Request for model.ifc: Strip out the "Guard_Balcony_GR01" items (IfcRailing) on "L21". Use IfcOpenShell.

First a look at what the model holds.

```python
import ifcopenshell
import ifcopenshell.util.element

model = ifcopenshell.open("model.ifc")
print(model.schema)
storey = next(s for s in model.by_type("IfcBuildingStorey") if s.Name == "L21")
railings = [e for e in ifcopenshell.util.element.get_decomposition(storey) if e.is_a("IfcRailing")]
seen = {}
for e in railings:
    element_type = ifcopenshell.util.element.get_type(e)
    name = element_type.Name if element_type not in (None, e) else None
    seen[name] = seen.get(name, 0) + 1
for name, count in sorted(seen.items(), key=str):
    print(count, "x", name)
```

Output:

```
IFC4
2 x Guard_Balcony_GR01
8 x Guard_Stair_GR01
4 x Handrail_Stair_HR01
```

```python
import ifcopenshell
import ifcopenshell.api.root
import ifcopenshell.util.element

model = ifcopenshell.open("model.ifc")

storey = next(s for s in model.by_type("IfcBuildingStorey") if s.Name == "L21")
railings = [e for e in ifcopenshell.util.element.get_decomposition(storey) if e.is_a("IfcRailing")]
targets = [e for e in railings if (t := ifcopenshell.util.element.get_type(e)) not in (None, e) and t.Name == "Guard_Balcony_GR01"]

for e in targets:
    ifcopenshell.api.root.remove_product(model, product=e)
print(len(targets), "removed")

model.write("model_edited.ifc")
```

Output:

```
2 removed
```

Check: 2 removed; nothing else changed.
